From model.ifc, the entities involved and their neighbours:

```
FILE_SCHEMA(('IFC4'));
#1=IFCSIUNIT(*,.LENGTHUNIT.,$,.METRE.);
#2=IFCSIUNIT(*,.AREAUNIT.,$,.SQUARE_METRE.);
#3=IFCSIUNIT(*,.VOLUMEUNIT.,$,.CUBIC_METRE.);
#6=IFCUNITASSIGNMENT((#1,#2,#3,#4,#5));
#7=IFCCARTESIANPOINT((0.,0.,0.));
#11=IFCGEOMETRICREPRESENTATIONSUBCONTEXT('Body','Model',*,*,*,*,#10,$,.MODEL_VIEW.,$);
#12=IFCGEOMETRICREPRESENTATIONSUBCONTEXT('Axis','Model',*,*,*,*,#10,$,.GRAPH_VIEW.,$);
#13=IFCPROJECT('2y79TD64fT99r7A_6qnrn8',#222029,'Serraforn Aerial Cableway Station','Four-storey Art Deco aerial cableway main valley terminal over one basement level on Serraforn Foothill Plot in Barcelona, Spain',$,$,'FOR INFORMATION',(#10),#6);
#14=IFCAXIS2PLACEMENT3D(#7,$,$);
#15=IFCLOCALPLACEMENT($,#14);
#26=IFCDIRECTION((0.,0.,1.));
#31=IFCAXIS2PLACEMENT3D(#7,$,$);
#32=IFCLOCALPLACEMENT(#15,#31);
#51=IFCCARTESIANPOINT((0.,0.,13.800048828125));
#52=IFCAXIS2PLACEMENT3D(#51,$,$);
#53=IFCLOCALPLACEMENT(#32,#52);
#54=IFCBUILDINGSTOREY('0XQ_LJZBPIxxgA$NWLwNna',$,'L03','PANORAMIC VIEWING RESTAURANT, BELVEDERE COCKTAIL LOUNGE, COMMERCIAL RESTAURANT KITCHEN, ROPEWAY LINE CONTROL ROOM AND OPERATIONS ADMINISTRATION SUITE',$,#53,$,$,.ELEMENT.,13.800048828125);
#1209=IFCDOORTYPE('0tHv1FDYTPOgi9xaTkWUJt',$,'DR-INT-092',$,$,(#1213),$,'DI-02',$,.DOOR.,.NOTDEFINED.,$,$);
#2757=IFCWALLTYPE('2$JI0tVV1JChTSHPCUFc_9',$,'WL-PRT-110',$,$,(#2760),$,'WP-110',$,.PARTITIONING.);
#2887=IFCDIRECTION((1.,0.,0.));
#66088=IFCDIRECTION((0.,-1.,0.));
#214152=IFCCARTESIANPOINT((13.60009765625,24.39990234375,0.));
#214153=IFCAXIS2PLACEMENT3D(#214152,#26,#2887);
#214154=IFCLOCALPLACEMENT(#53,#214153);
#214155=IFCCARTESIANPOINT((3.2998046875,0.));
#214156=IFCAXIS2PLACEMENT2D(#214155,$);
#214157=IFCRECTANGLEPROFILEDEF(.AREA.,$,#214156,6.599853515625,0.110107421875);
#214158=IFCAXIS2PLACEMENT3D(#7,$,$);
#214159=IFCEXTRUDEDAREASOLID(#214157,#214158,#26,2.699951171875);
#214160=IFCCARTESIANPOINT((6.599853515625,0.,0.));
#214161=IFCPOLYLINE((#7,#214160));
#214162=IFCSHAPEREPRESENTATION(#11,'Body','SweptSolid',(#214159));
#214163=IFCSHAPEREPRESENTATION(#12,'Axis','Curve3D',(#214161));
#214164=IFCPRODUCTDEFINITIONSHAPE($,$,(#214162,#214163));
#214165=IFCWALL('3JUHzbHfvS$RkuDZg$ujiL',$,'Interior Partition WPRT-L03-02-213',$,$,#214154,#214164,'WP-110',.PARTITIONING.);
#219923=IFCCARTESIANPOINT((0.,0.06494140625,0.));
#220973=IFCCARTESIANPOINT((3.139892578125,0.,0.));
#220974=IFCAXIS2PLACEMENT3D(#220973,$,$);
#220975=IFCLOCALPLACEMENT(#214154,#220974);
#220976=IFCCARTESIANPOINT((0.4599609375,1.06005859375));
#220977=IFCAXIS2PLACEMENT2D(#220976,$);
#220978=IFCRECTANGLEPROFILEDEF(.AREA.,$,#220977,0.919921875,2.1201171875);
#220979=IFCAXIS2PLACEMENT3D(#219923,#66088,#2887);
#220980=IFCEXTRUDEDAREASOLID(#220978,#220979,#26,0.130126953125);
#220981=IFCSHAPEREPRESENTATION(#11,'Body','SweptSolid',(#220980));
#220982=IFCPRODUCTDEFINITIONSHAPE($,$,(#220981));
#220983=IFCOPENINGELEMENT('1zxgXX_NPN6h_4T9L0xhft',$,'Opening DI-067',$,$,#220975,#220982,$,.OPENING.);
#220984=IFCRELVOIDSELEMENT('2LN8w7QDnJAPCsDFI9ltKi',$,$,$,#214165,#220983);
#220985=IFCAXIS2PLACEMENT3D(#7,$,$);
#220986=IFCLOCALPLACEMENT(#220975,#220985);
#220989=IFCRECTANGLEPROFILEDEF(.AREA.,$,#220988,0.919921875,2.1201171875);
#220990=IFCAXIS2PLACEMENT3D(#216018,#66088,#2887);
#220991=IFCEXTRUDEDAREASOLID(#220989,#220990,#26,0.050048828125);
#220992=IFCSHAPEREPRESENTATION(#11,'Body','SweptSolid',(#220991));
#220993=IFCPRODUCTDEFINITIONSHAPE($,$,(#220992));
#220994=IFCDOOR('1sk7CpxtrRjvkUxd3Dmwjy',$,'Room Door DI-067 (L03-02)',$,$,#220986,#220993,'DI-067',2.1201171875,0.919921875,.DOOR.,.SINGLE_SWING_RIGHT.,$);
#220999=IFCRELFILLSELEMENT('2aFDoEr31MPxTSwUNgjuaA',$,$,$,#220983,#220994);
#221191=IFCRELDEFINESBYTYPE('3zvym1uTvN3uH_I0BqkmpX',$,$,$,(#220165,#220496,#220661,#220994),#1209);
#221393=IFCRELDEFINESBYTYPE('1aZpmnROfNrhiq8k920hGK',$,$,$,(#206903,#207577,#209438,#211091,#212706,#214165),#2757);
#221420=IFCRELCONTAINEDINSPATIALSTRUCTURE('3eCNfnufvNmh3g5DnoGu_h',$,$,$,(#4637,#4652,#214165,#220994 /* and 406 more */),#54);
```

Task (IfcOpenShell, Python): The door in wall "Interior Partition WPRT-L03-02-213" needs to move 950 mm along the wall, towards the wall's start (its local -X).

```python
import ifcopenshell
import ifcopenshell.api.geometry
import ifcopenshell.util.placement

model = ifcopenshell.open("model.ifc")

door = model.by_guid("1sk7CpxtrRjvkUxd3Dmwjy")
opening = door.FillsVoids[0].RelatingOpeningElement
wall = opening.VoidsElements[0].RelatingBuildingElement

wall_matrix = ifcopenshell.util.placement.get_local_placement(wall.ObjectPlacement)
shift = wall_matrix[:3, 0] * -0.95
before = ifcopenshell.util.placement.get_local_placement(door.ObjectPlacement)[:3, 3].copy()

# The door is placed relative to its opening, so it follows when the opening moves.
matrix = ifcopenshell.util.placement.get_local_placement(opening.ObjectPlacement)
matrix[:3, 3] += shift
ifcopenshell.api.geometry.edit_object_placement(
    model, product=opening, matrix=matrix, is_si=False, should_transform_children=True
)

after = ifcopenshell.util.placement.get_local_placement(door.ObjectPlacement)[:3, 3]
print("door moved by", (after - before).round(3) + 0.0)

model.write("model_edited.ifc")
```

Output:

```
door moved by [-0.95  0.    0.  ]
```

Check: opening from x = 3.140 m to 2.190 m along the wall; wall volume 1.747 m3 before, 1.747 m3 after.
